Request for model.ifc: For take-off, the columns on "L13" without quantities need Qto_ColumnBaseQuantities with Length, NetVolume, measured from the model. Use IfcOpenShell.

First a look at what the model holds.

```python
import ifcopenshell
import ifcopenshell.util.element
import ifcopenshell.util.unit

model = ifcopenshell.open("model.ifc")
print(model.schema)
for unit_type in ("LENGTHUNIT", "AREAUNIT", "VOLUMEUNIT"):
    print(unit_type, ifcopenshell.util.unit.calculate_unit_scale(model, unit_type))
storey = next(s for s in model.by_type("IfcBuildingStorey") if s.Name == "L13")
columns = [e for e in ifcopenshell.util.element.get_decomposition(storey) if e.is_a("IfcColumn")]
for e in sorted(columns, key=lambda e: e.id()):
    print(e.id(), e.is_a(), e.Name, list(ifcopenshell.util.element.get_psets(e, qtos_only=True)), sep=" | ")
```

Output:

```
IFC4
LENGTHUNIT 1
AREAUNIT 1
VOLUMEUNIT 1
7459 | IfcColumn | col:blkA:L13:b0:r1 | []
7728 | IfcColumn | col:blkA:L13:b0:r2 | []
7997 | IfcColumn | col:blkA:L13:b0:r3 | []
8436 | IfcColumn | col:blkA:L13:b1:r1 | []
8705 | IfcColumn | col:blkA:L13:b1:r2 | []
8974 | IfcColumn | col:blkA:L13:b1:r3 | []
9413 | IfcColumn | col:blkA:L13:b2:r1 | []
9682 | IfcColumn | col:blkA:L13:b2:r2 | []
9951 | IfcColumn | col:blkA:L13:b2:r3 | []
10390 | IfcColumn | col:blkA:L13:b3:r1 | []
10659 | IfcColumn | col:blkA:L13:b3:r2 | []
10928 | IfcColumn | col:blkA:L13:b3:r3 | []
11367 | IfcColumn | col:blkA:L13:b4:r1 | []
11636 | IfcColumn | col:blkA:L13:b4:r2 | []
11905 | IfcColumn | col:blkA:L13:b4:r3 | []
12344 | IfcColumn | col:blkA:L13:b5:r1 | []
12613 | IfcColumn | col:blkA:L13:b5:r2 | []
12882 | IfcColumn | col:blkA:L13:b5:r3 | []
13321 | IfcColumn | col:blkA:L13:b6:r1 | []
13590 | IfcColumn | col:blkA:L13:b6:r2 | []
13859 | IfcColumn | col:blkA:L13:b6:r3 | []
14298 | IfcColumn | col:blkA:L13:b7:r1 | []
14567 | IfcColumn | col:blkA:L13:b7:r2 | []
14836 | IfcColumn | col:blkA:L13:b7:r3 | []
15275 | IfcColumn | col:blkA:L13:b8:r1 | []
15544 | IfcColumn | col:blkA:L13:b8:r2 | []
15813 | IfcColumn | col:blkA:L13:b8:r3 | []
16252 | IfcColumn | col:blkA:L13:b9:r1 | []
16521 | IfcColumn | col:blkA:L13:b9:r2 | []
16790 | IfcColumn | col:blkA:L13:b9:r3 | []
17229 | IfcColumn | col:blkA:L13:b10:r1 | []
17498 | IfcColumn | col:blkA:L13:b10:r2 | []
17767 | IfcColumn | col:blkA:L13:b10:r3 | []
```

```python
import ifcopenshell
import ifcopenshell.api.pset
import ifcopenshell.geom
import ifcopenshell.util.element
import ifcopenshell.util.shape
import ifcopenshell.util.unit

model = ifcopenshell.open("model.ifc")
unit_scale = ifcopenshell.util.unit.calculate_unit_scale(model)
volume_scale = ifcopenshell.util.unit.calculate_unit_scale(model, "VOLUMEUNIT")
settings = ifcopenshell.geom.settings()

storey = next(s for s in model.by_type("IfcBuildingStorey") if s.Name == "L13")
columns = [e for e in ifcopenshell.util.element.get_decomposition(storey) if e.is_a("IfcColumn")]

for e in sorted(columns, key=lambda e: e.id()):
    if ifcopenshell.util.element.get_psets(e, qtos_only=True, should_inherit=False):
        continue
    # Geometry comes back in metres, in the element's own axes.
    shape = ifcopenshell.geom.create_shape(settings, e)
    values = {
        "Length": ifcopenshell.util.shape.get_z(shape.geometry) / unit_scale,
        "NetVolume": ifcopenshell.util.shape.get_volume(shape.geometry) / volume_scale,
    }
    qto = ifcopenshell.api.pset.add_qto(model, product=e, name="Qto_ColumnBaseQuantities")
    ifcopenshell.api.pset.edit_qto(model, qto=qto, properties=values)
    print(e.id(), {k: round(v, 3) for k, v in values.items()})

model.write("model_updated.ifc")
```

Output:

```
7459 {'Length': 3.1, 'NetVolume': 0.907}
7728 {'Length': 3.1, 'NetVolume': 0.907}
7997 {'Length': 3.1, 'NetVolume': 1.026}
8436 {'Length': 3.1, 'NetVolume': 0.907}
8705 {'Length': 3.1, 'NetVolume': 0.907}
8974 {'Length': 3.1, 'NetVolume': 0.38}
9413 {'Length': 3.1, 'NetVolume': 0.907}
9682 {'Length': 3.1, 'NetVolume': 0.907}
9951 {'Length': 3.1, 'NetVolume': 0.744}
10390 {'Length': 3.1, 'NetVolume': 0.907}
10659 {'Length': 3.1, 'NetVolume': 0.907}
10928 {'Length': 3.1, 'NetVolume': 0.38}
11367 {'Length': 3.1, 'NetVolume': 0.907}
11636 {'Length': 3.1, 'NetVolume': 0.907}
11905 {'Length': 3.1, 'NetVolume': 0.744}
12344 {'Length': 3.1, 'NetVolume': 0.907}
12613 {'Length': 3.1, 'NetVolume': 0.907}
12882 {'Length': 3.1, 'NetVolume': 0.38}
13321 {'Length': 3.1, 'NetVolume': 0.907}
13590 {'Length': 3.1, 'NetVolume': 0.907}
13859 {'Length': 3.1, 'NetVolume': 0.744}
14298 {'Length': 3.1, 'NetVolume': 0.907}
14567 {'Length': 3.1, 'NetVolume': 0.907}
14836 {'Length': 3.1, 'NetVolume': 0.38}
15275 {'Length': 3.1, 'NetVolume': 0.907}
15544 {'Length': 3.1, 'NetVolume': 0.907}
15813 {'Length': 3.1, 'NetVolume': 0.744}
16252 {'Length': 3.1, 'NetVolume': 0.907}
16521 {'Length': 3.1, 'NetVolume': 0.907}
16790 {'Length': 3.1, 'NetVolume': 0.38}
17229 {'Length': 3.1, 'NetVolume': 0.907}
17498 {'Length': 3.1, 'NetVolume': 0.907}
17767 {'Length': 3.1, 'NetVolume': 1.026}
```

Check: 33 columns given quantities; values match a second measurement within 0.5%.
